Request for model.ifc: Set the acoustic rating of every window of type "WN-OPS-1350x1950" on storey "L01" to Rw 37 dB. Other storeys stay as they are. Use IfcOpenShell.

First a look at what the model holds.

```python
import ifcopenshell
import ifcopenshell.util.element

model = ifcopenshell.open("model.ifc")
print(model.schema)
storey = next(s for s in model.by_type("IfcBuildingStorey") if s.Name == "L01")
windows = [e for e in ifcopenshell.util.element.get_decomposition(storey) if e.is_a("IfcWindow")]
seen = {}
for e in windows:
    element_type = ifcopenshell.util.element.get_type(e)
    key = (element_type.Name if element_type != e and element_type else None, ifcopenshell.util.element.get_pset(e, "Pset_WindowCommon", "AcousticRating"))
    seen[key] = seen.get(key, 0) + 1
for (name, value), count in sorted(seen.items(), key=str):
    print(count, "x", name, "|", value)
```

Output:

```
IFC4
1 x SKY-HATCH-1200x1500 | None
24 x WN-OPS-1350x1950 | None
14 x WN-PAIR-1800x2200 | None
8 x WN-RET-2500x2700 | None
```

```python
import ifcopenshell
import ifcopenshell.api.pset
import ifcopenshell.util.element

model = ifcopenshell.open("model.ifc")

storey = next(s for s in model.by_type("IfcBuildingStorey") if s.Name == "L01")
windows = [e for e in ifcopenshell.util.element.get_decomposition(storey) if e.is_a("IfcWindow")]

count = 0
for e in windows:
    element_type = ifcopenshell.util.element.get_type(e)
    if element_type in (None, e) or element_type.Name != "WN-OPS-1350x1950":
        continue
    # add_pset returns the element's existing set when there is one.
    pset = ifcopenshell.api.pset.add_pset(model, product=e, name="Pset_WindowCommon")
    ifcopenshell.api.pset.edit_pset(model, pset=pset, properties={"AcousticRating": "Rw 37 dB"})
    count += 1

print(count, "windows updated")

model.write("model_v2.ifc")
```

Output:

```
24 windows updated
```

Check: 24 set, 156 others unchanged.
